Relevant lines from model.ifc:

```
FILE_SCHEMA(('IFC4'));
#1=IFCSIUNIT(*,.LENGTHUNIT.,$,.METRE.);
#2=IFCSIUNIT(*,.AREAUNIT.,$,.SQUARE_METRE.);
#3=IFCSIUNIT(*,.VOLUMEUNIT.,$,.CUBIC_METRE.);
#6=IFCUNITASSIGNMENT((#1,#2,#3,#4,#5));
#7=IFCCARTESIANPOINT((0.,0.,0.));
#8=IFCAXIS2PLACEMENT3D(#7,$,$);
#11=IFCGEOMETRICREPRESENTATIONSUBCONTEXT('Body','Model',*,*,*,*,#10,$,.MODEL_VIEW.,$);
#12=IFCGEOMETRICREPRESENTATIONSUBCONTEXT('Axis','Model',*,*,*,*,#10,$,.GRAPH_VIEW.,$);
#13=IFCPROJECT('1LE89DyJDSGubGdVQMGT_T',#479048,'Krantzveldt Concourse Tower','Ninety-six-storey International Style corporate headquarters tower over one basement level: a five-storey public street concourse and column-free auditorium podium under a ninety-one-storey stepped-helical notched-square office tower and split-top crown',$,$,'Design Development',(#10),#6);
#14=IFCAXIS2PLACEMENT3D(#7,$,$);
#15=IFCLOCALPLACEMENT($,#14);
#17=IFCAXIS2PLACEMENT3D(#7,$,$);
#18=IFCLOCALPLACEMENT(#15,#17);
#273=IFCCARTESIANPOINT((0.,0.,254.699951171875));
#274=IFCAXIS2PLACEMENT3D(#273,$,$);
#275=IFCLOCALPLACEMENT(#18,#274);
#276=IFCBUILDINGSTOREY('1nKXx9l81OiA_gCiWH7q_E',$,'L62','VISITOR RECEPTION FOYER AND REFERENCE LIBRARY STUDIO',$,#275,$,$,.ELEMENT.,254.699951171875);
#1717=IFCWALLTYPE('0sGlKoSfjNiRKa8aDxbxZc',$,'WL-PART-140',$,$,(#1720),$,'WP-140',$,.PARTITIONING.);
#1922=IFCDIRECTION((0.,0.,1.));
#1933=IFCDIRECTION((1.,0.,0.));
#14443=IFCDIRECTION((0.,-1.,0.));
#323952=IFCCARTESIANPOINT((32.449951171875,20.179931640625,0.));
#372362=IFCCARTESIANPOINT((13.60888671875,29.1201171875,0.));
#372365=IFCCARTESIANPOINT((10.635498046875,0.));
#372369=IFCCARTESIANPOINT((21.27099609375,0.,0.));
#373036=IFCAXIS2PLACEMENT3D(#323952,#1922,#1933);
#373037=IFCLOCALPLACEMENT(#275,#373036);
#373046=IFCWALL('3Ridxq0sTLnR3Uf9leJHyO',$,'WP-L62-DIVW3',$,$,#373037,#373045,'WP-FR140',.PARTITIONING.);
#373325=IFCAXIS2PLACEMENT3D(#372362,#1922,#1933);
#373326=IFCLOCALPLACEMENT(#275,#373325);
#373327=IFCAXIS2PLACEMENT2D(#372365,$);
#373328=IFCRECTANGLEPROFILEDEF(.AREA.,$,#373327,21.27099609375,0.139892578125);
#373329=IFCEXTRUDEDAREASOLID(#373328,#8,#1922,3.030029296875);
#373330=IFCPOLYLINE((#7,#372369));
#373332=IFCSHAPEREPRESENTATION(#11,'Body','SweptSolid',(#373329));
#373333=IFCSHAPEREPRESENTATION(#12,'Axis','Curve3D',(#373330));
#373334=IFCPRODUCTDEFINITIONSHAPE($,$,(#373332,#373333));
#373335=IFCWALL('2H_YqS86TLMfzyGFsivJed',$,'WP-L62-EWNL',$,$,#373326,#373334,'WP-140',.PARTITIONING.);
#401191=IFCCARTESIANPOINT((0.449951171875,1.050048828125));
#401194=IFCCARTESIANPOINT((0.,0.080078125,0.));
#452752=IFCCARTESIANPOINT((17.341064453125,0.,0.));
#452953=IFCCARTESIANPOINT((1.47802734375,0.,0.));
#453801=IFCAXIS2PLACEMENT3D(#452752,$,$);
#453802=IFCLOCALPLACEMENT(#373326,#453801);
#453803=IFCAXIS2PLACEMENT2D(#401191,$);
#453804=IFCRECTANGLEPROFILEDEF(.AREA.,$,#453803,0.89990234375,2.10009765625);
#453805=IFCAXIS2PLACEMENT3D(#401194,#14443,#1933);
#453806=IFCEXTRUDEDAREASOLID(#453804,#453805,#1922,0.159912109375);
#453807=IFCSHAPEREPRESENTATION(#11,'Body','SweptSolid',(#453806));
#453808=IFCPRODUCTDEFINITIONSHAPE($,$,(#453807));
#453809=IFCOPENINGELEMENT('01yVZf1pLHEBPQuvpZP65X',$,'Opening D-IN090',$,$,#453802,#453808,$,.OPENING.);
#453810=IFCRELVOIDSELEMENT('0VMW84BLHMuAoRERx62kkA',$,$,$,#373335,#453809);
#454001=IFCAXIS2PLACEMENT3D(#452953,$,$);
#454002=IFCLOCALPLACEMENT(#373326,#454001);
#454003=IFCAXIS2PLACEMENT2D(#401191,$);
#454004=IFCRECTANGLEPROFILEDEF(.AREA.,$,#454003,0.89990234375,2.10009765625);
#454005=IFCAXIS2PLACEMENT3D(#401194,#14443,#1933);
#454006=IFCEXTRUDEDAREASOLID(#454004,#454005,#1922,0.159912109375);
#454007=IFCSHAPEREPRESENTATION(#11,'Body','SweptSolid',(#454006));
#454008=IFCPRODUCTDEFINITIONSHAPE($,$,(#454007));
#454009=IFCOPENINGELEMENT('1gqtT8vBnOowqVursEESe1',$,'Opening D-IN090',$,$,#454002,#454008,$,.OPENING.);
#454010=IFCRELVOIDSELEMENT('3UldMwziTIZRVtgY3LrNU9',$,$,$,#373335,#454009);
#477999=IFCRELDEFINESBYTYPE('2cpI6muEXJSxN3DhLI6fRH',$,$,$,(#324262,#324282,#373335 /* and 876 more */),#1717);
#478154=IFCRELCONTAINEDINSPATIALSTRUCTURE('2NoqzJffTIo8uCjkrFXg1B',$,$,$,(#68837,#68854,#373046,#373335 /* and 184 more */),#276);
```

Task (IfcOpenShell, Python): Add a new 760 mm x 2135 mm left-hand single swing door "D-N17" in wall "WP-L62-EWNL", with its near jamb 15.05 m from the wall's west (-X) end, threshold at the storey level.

```python
import numpy as np
import ifcopenshell
import ifcopenshell.api.feature
import ifcopenshell.api.geometry
import ifcopenshell.api.root
import ifcopenshell.api.spatial
import ifcopenshell.geom
import ifcopenshell.util.element
import ifcopenshell.util.placement
import ifcopenshell.util.representation
import ifcopenshell.util.shape
import ifcopenshell.util.unit

model = ifcopenshell.open("model.ifc")
unit_scale = ifcopenshell.util.unit.calculate_unit_scale(model)
settings = ifcopenshell.geom.settings()


def volume(element):
    """Net volume in cubic metres, openings subtracted."""
    shape = ifcopenshell.geom.create_shape(settings, element)
    return ifcopenshell.util.shape.get_volume(shape.geometry)


wall = model.by_guid("2H_YqS86TLMfzyGFsivJed")
storey = ifcopenshell.util.element.get_container(wall, ifc_class="IfcBuildingStorey")
context = ifcopenshell.util.representation.get_context(model, "Model", "Body", "MODEL_VIEW")
before = volume(wall)

width, height, from_end, sill = 0.76, 2.135, 15.05, 0.0  # metres

# The wall runs along its own X axis, and the end named is its -X end.
wall_shape = ifcopenshell.geom.create_shape(settings, wall)
x, y, z = ifcopenshell.util.shape.get_vertices(wall_shape.geometry).T
start = x.min() + from_end
face, thickness = float(y.min()), float(y.max() - y.min())
wall_matrix = ifcopenshell.util.placement.get_local_placement(wall.ObjectPlacement)
level = ifcopenshell.util.placement.get_local_placement(storey.ObjectPlacement)[2, 3]


def in_wall(x, y):
    """Placement at x, y metres in the wall's axes, at sill height."""
    matrix = wall_matrix.copy()
    matrix[:, 3] = wall_matrix @ np.array([x / unit_scale, y / unit_scale, 0.0, 1.0])
    matrix[2, 3] = level + sill / unit_scale
    return matrix


# Opening: a box that overshoots both wall faces by 50 mm.
opening = ifcopenshell.api.root.create_entity(model, ifc_class="IfcOpeningElement", predefined_type="OPENING")
box = ifcopenshell.api.geometry.add_wall_representation(
    model, context=context, length=width, height=height, thickness=thickness + 0.1
)
ifcopenshell.api.geometry.assign_representation(model, product=opening, representation=box)
ifcopenshell.api.geometry.edit_object_placement(model, product=opening, matrix=in_wall(start, face - 0.05), is_si=False)
ifcopenshell.api.feature.add_feature(model, feature=opening, element=wall)

door = ifcopenshell.api.root.create_entity(model, ifc_class="IfcDoor", name="D-N17", predefined_type="DOOR")
door.OverallWidth, door.OverallHeight = width / unit_scale, height / unit_scale
door.OperationType = "SINGLE_SWING_LEFT"
body = ifcopenshell.api.geometry.add_door_representation(
    model,
    context=context,
    overall_width=door.OverallWidth,
    overall_height=door.OverallHeight,
    operation_type="SINGLE_SWING_LEFT",
    lining_properties={"LiningDepth": thickness / unit_scale, "ThresholdDepth": thickness / unit_scale},
)
ifcopenshell.api.geometry.assign_representation(model, product=door, representation=body)
ifcopenshell.api.spatial.assign_container(model, products=[door], relating_structure=storey)
ifcopenshell.api.feature.add_filling(model, opening=opening, element=door)

# The lining spans the wall, so the door starts at the wall face.
ifcopenshell.api.geometry.edit_object_placement(model, product=door, matrix=in_wall(start, face), is_si=False)

after = volume(wall)

print(f"wall volume {before:.3f} -> {after:.3f} m3")

model.write("model_rev.ifc")
```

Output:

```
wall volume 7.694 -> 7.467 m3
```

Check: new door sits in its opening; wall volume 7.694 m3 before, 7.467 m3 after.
